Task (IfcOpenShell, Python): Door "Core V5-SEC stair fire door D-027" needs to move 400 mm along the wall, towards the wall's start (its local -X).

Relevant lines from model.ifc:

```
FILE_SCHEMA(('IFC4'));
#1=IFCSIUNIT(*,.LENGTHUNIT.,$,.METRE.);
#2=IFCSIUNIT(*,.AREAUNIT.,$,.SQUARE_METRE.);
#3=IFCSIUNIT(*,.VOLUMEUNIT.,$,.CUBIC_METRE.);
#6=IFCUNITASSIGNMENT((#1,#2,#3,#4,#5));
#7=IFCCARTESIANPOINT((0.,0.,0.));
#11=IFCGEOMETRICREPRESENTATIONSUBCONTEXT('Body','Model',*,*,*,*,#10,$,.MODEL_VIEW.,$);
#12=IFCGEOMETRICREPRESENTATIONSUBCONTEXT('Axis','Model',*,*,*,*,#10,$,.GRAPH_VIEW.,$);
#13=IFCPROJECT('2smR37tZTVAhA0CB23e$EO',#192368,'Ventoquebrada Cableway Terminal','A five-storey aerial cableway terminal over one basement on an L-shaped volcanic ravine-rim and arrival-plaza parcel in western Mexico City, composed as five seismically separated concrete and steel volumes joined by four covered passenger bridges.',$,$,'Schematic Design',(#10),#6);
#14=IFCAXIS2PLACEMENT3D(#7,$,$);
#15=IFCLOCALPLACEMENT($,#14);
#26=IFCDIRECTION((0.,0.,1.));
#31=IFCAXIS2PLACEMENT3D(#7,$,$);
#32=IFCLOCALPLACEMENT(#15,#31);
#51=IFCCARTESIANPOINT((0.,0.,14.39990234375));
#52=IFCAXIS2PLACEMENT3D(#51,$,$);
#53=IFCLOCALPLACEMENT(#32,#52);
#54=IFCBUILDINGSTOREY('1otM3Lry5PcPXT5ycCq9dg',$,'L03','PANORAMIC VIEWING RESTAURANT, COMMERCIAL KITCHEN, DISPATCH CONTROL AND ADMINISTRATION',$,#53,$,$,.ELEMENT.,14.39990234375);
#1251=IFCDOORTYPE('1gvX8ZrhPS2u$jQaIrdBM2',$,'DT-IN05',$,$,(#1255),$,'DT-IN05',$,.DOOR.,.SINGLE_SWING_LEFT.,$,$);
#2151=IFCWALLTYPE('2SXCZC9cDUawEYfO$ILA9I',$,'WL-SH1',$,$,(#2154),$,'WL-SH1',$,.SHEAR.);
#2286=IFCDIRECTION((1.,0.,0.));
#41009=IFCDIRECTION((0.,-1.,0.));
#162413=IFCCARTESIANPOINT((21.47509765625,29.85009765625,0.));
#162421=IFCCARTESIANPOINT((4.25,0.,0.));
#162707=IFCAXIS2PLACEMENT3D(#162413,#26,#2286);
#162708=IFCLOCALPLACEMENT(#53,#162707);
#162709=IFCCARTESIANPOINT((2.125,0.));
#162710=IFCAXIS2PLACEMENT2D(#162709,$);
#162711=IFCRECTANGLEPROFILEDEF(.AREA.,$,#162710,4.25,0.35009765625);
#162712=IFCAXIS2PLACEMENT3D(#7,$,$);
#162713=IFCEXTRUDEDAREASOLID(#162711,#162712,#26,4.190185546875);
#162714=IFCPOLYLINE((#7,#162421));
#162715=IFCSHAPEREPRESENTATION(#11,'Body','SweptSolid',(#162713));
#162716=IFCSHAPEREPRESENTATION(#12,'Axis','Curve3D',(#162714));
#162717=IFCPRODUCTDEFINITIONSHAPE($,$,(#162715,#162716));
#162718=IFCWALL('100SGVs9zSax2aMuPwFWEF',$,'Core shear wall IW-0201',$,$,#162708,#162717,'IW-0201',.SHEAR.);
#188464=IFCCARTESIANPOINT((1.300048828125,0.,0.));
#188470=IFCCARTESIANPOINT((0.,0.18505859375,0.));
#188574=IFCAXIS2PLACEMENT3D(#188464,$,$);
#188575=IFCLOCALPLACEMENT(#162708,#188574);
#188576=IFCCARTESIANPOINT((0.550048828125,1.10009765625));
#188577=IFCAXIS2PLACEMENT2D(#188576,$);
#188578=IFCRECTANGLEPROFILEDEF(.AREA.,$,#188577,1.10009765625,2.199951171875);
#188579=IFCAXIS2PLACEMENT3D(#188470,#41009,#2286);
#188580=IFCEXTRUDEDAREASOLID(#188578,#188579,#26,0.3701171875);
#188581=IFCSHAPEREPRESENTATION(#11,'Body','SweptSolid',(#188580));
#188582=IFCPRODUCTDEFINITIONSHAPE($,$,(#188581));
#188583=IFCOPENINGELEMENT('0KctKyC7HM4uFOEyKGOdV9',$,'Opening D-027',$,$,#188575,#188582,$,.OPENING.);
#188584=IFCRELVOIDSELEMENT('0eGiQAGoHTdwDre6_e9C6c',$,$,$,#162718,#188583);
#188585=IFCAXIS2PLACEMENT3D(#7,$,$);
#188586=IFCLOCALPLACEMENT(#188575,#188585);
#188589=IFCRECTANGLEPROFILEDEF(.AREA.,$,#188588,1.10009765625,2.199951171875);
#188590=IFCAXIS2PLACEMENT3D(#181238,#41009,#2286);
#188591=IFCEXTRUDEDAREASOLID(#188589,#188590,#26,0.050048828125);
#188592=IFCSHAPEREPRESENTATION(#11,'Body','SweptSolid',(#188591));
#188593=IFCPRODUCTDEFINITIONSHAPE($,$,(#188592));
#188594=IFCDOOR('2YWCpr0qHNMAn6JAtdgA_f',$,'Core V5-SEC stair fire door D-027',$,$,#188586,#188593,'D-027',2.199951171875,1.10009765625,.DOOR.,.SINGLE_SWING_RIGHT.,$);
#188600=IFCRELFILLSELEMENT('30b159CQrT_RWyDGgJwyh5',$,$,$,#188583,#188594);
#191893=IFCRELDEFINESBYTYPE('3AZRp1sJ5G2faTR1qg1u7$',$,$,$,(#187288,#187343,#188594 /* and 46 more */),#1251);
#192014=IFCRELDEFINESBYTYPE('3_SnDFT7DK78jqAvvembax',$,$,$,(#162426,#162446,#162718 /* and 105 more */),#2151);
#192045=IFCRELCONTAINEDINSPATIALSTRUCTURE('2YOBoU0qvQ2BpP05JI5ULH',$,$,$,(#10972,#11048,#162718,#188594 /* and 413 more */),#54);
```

```python
import ifcopenshell
import ifcopenshell.api.geometry
import ifcopenshell.util.placement
import ifcopenshell.util.unit

model = ifcopenshell.open("model.ifc")
unit_scale = ifcopenshell.util.unit.calculate_unit_scale(model)

door = model.by_guid("2YWCpr0qHNMAn6JAtdgA_f")
opening = door.FillsVoids[0].RelatingOpeningElement
wall = opening.VoidsElements[0].RelatingBuildingElement

wall_matrix = ifcopenshell.util.placement.get_local_placement(wall.ObjectPlacement)
shift = wall_matrix[:3, 0] * -0.4 / unit_scale
before = ifcopenshell.util.placement.get_local_placement(door.ObjectPlacement)[:3, 3].copy()

# The door is placed relative to its opening, so it follows when the opening moves.
matrix = ifcopenshell.util.placement.get_local_placement(opening.ObjectPlacement)
matrix[:3, 3] += shift
ifcopenshell.api.geometry.edit_object_placement(
    model, product=opening, matrix=matrix, is_si=False, should_transform_children=True
)

after = ifcopenshell.util.placement.get_local_placement(door.ObjectPlacement)[:3, 3]
print("door moved by", (after - before).round(3) + 0.0)

model.write("model_v2.ifc")
```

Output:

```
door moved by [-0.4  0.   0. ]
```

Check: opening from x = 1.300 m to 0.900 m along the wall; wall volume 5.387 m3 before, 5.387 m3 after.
